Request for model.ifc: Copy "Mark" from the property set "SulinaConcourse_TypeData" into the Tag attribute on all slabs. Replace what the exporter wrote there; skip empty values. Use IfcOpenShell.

First a look at what the model holds.

```python
import ifcopenshell
import ifcopenshell.util.element

model = ifcopenshell.open("model.ifc")
print(model.schema)
slabs = model.by_type("IfcSlab")
print(len(slabs), "slabs")
for e in slabs[:8]:
    source = ifcopenshell.util.element.get_pset(e, "SulinaConcourse_TypeData", "Mark")
    target = e.Tag
    print(e.id(), repr(source), repr(target), sep=" | ")
```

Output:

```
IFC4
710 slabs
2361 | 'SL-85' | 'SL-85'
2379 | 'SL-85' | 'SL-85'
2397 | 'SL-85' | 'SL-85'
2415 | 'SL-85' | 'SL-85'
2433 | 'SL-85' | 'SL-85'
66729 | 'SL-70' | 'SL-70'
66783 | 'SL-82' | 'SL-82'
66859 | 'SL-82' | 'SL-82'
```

```python
import ifcopenshell
import ifcopenshell.util.element

model = ifcopenshell.open("model.ifc")

count = 0
for e in model.by_type("IfcSlab"):
    value = ifcopenshell.util.element.get_pset(e, "SulinaConcourse_TypeData", "Mark")
    current = e.Tag
    if not value or not value.strip() or current == value:
        continue
    e.Tag = value
    count += 1

print(count, "slabs updated")

model.write("model_rev.ifc")
```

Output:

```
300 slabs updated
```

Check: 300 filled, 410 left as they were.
